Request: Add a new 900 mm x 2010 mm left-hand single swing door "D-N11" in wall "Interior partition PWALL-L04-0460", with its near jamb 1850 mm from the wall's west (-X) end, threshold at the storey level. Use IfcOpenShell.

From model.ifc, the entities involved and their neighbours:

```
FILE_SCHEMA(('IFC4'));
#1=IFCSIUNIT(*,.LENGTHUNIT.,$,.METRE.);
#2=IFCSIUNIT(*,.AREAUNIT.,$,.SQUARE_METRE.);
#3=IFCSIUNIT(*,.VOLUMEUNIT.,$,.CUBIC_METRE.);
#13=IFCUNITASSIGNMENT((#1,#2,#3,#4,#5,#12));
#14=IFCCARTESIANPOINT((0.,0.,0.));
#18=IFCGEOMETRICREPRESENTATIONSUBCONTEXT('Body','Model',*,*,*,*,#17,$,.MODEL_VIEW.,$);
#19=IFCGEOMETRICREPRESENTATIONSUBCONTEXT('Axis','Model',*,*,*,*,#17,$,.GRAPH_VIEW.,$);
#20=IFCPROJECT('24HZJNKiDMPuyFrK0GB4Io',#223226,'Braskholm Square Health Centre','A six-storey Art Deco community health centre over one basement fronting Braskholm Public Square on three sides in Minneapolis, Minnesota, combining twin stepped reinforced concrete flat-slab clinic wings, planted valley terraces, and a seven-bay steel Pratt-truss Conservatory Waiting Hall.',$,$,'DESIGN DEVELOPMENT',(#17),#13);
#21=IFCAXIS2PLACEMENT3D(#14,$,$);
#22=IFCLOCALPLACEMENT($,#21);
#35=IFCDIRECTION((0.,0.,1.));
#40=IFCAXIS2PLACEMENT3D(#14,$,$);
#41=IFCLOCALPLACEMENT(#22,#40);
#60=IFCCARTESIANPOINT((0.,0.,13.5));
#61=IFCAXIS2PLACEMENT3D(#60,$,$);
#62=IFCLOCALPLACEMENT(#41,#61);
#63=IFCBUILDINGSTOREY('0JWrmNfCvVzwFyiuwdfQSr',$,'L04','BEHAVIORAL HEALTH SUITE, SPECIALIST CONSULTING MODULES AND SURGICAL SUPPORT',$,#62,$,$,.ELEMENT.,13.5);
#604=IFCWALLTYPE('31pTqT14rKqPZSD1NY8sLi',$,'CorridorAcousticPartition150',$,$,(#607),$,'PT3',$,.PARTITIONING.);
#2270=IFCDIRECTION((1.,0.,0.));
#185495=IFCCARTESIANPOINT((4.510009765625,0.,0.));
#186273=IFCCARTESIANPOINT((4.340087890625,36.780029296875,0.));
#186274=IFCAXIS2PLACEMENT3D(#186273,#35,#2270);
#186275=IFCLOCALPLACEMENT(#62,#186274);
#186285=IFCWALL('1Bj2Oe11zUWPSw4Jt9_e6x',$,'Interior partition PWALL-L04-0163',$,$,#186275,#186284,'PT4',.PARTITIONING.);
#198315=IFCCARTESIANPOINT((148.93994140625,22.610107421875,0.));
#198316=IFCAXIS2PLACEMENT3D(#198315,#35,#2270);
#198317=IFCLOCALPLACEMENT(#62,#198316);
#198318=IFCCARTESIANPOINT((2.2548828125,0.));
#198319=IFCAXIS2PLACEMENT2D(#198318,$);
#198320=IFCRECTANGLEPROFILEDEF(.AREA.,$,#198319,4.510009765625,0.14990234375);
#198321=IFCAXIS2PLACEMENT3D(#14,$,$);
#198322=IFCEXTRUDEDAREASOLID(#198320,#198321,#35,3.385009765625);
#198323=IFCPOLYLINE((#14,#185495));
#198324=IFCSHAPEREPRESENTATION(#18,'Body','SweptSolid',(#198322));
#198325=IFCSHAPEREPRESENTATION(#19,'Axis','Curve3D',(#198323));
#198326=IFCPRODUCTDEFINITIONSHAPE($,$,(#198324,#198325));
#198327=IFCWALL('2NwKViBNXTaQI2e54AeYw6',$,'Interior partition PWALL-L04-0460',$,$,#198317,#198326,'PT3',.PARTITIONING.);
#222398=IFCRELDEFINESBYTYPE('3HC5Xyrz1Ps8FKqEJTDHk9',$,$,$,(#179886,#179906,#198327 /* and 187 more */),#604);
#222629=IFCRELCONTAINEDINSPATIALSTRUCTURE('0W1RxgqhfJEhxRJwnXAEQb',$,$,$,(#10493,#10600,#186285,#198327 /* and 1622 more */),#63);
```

```python
import numpy as np
import ifcopenshell
import ifcopenshell.api.feature
import ifcopenshell.api.geometry
import ifcopenshell.api.root
import ifcopenshell.api.spatial
import ifcopenshell.geom
import ifcopenshell.util.element
import ifcopenshell.util.placement
import ifcopenshell.util.representation
import ifcopenshell.util.shape
import ifcopenshell.util.unit

model = ifcopenshell.open("model.ifc")
unit_scale = ifcopenshell.util.unit.calculate_unit_scale(model)
settings = ifcopenshell.geom.settings()


def volume(element):
    """Net volume in cubic metres, openings subtracted."""
    shape = ifcopenshell.geom.create_shape(settings, element)
    return ifcopenshell.util.shape.get_volume(shape.geometry)


wall = model.by_id(198327)
storey = ifcopenshell.util.element.get_container(wall, ifc_class="IfcBuildingStorey")
context = ifcopenshell.util.representation.get_context(model, "Model", "Body", "MODEL_VIEW")
before = volume(wall)

width, height, from_end, sill = 0.9, 2.01, 1.85, 0.0  # metres

# The wall runs along its own X axis, and the end named is its -X end.
wall_shape = ifcopenshell.geom.create_shape(settings, wall)
x, y, z = ifcopenshell.util.shape.get_vertices(wall_shape.geometry).T
start = x.min() + from_end
face, thickness = float(y.min()), float(y.max() - y.min())
wall_matrix = ifcopenshell.util.placement.get_local_placement(wall.ObjectPlacement)
level = ifcopenshell.util.placement.get_local_placement(storey.ObjectPlacement)[2, 3]


def in_wall(x, y):
    """Placement at x, y metres in the wall's axes, at sill height."""
    matrix = wall_matrix.copy()
    matrix[:, 3] = wall_matrix @ np.array([x / unit_scale, y / unit_scale, 0.0, 1.0])
    matrix[2, 3] = level + sill / unit_scale
    return matrix


# Opening: a box that overshoots both wall faces by 50 mm.
opening = ifcopenshell.api.root.create_entity(model, ifc_class="IfcOpeningElement", predefined_type="OPENING")
box = ifcopenshell.api.geometry.add_wall_representation(
    model, context=context, length=width, height=height, thickness=thickness + 0.1
)
ifcopenshell.api.geometry.assign_representation(model, product=opening, representation=box)
ifcopenshell.api.geometry.edit_object_placement(model, product=opening, matrix=in_wall(start, face - 0.05), is_si=False)
ifcopenshell.api.feature.add_feature(model, feature=opening, element=wall)

door = ifcopenshell.api.root.create_entity(model, ifc_class="IfcDoor", name="D-N11", predefined_type="DOOR")
door.OverallWidth, door.OverallHeight = width / unit_scale, height / unit_scale
door.OperationType = "SINGLE_SWING_LEFT"
body = ifcopenshell.api.geometry.add_door_representation(
    model,
    context=context,
    overall_width=door.OverallWidth,
    overall_height=door.OverallHeight,
    operation_type="SINGLE_SWING_LEFT",
    lining_properties={"LiningDepth": thickness / unit_scale, "ThresholdDepth": thickness / unit_scale},
)
ifcopenshell.api.geometry.assign_representation(model, product=door, representation=body)
ifcopenshell.api.spatial.assign_container(model, products=[door], relating_structure=storey)
ifcopenshell.api.feature.add_filling(model, opening=opening, element=door)

# The lining spans the wall, so the door starts at the wall face.
ifcopenshell.api.geometry.edit_object_placement(model, product=door, matrix=in_wall(start, face), is_si=False)

after = volume(wall)

print(f"wall volume {before:.3f} -> {after:.3f} m3")

model.write("model_edited.ifc")
```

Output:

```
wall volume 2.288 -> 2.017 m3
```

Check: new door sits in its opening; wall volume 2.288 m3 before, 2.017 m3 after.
